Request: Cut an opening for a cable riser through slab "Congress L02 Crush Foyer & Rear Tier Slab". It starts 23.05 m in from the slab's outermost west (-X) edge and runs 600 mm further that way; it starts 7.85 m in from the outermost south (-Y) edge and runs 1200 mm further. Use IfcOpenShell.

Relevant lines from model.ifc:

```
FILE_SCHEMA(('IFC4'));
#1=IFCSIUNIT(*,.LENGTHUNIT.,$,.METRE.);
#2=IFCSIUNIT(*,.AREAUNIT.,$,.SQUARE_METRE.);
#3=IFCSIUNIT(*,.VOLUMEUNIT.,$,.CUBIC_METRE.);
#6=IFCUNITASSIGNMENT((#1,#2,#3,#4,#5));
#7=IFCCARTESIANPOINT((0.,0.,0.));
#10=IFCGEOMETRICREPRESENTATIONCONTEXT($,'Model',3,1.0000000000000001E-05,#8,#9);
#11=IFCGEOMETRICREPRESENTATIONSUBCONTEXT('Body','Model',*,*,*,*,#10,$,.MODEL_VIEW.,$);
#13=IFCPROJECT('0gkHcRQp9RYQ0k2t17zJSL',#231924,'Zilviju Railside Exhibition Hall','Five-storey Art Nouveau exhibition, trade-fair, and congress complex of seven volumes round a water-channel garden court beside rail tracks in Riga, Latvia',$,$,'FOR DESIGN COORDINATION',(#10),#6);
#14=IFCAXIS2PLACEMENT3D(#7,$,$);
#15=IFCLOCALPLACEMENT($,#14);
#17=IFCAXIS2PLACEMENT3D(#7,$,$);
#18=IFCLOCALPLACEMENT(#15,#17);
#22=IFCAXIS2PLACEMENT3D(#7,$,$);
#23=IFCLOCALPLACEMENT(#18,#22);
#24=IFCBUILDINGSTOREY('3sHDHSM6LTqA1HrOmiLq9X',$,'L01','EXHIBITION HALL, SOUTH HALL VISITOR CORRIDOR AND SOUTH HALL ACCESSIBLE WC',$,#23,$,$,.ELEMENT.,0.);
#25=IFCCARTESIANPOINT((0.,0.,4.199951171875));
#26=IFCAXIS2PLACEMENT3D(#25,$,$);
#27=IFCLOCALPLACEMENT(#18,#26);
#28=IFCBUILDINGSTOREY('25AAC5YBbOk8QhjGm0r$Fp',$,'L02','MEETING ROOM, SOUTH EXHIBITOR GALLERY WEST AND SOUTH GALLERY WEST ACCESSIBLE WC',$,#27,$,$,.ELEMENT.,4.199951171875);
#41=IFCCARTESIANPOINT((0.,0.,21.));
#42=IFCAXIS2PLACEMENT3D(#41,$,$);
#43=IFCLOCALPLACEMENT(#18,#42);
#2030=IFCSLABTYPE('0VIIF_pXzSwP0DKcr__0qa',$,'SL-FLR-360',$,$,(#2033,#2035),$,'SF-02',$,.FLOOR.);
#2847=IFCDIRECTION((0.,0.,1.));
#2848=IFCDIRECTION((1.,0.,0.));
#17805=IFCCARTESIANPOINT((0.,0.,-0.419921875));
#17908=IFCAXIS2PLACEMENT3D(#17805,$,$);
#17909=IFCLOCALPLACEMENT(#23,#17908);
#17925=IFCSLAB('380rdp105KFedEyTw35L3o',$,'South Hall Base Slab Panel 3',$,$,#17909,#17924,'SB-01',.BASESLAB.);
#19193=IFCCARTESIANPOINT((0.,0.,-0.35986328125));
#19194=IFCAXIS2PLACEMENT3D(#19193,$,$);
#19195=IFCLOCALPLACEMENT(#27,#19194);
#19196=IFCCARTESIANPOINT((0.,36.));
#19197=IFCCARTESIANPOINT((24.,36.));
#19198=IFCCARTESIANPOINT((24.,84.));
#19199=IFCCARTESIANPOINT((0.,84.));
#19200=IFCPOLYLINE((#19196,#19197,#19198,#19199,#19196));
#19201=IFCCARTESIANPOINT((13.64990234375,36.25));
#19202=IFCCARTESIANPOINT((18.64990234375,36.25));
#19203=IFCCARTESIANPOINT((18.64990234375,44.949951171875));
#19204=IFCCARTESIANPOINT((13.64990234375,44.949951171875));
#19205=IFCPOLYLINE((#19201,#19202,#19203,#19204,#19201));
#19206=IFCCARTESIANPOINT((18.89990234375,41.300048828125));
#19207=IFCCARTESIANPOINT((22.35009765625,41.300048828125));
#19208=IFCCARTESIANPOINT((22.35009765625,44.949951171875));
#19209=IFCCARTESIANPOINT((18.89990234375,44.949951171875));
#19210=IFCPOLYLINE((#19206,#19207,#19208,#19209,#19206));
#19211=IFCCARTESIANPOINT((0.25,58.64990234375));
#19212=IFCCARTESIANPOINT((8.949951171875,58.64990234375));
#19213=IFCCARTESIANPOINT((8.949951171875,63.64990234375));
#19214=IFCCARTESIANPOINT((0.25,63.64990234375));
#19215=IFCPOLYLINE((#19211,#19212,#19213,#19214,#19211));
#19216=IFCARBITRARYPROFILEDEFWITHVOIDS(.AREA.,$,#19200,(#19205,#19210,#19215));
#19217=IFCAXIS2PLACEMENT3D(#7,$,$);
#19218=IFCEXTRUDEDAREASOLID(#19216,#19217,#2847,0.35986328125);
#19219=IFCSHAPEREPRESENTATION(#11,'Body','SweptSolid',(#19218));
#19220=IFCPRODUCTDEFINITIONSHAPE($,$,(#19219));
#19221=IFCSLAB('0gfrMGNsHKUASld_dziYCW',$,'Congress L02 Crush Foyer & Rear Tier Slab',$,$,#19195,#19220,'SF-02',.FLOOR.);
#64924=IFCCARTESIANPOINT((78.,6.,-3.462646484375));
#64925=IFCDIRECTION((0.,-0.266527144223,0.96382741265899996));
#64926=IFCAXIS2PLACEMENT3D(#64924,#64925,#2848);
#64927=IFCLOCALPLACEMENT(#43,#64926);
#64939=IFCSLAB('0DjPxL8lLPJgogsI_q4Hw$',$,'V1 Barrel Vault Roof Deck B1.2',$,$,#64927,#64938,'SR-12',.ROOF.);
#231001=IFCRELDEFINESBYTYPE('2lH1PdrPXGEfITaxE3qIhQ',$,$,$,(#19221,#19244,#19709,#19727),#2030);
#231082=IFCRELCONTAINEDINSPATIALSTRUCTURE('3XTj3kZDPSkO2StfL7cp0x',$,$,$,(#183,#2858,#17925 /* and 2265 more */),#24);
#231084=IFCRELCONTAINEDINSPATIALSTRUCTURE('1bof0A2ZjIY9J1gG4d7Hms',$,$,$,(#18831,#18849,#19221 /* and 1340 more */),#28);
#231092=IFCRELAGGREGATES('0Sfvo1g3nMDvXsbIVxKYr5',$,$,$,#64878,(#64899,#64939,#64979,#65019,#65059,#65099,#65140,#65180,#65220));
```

```python
import numpy as np
import ifcopenshell
import ifcopenshell.api.feature
import ifcopenshell.api.geometry
import ifcopenshell.api.root
import ifcopenshell.geom
import ifcopenshell.util.placement
import ifcopenshell.util.representation
import ifcopenshell.util.shape
import ifcopenshell.util.unit

model = ifcopenshell.open("model.ifc")
unit_scale = ifcopenshell.util.unit.calculate_unit_scale(model)
settings = ifcopenshell.geom.settings()


def volume(element):
    """Net volume in cubic metres, openings subtracted."""
    shape = ifcopenshell.geom.create_shape(settings, element)
    return ifcopenshell.util.shape.get_volume(shape.geometry)


slab = model.by_guid("0gfrMGNsHKUASld_dziYCW")
before = volume(slab)

# Extent in the slab's own axes, in metres. The edges named are its -X and -Y sides.
slab_shape = ifcopenshell.geom.create_shape(settings, slab)
vertices = ifcopenshell.util.shape.get_vertices(slab_shape.geometry)
x_min, y_min, bottom = vertices.min(axis=0)
top = vertices[:, 2].max()

opening = ifcopenshell.api.root.create_entity(model, ifc_class="IfcOpeningElement", name="Cable riser opening", predefined_type="OPENING")
context = ifcopenshell.util.representation.get_context(model, "Model", "Body", "MODEL_VIEW")
width, depth = 0.6, 1.2
outline = [(0.0, 0.0), (width, 0.0), (width, depth), (0.0, depth), (0.0, 0.0)]
# Overshoot both faces by 50 mm so the cut is clean.
shape = ifcopenshell.api.geometry.add_slab_representation(
    model, context=context, depth=top - bottom + 0.1, polyline=outline
)
ifcopenshell.api.geometry.assign_representation(model, product=opening, representation=shape)

matrix = ifcopenshell.util.placement.get_local_placement(slab.ObjectPlacement)
matrix[:, 3] = matrix @ np.append(np.array([x_min + 23.05, y_min + 7.85, bottom - 0.05]) / unit_scale, 1.0)
ifcopenshell.api.geometry.edit_object_placement(model, product=opening, matrix=matrix, is_si=False)
ifcopenshell.api.feature.add_feature(model, feature=opening, element=slab)

after = volume(slab)

print(f"slab volume {before:.3f} -> {after:.3f} m3")

model.write("model_v2.ifc")
```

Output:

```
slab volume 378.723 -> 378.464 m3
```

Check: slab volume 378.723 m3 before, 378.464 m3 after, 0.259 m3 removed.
